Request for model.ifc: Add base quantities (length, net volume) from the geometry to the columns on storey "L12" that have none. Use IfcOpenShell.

First a look at what the model holds.

```python
import ifcopenshell
import ifcopenshell.util.element
import ifcopenshell.util.unit

model = ifcopenshell.open("model.ifc")
print(model.schema)
for unit_type in ("LENGTHUNIT", "AREAUNIT", "VOLUMEUNIT"):
    print(unit_type, ifcopenshell.util.unit.calculate_unit_scale(model, unit_type))
storey = next(s for s in model.by_type("IfcBuildingStorey") if s.Name == "L12")
columns = [e for e in ifcopenshell.util.element.get_decomposition(storey) if e.is_a("IfcColumn")]
for e in sorted(columns, key=lambda e: e.id()):
    print(e.id(), e.is_a(), e.Name, list(ifcopenshell.util.element.get_psets(e, qtos_only=True)), sep=" | ")
```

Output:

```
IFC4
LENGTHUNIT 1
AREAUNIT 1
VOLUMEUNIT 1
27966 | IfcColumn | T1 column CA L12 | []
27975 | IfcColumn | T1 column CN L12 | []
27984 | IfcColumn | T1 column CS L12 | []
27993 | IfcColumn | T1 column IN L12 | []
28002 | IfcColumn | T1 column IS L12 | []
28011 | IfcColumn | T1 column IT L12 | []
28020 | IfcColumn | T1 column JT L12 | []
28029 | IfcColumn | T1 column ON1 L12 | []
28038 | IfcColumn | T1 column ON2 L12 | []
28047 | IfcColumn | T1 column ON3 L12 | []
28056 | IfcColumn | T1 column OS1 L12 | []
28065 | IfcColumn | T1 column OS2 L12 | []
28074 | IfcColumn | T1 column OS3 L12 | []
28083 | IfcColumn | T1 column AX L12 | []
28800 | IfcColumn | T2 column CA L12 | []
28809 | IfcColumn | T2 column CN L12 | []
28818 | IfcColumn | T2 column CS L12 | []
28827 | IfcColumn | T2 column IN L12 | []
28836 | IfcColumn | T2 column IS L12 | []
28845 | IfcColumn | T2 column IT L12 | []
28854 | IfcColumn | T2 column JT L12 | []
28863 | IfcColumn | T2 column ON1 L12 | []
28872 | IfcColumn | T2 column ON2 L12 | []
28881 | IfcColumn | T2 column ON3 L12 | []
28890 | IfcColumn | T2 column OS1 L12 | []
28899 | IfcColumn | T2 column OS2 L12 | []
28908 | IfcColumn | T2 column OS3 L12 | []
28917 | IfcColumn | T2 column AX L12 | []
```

```python
import ifcopenshell
import ifcopenshell.api.pset
import ifcopenshell.geom
import ifcopenshell.util.element
import ifcopenshell.util.shape
import ifcopenshell.util.unit

model = ifcopenshell.open("model.ifc")
unit_scale = ifcopenshell.util.unit.calculate_unit_scale(model)
volume_scale = ifcopenshell.util.unit.calculate_unit_scale(model, "VOLUMEUNIT")
settings = ifcopenshell.geom.settings()

storey = next(s for s in model.by_type("IfcBuildingStorey") if s.Name == "L12")
columns = [e for e in ifcopenshell.util.element.get_decomposition(storey) if e.is_a("IfcColumn")]

for e in sorted(columns, key=lambda e: e.id()):
    if ifcopenshell.util.element.get_psets(e, qtos_only=True, should_inherit=False):
        continue
    # Geometry comes back in metres, in the element's own axes.
    shape = ifcopenshell.geom.create_shape(settings, e)
    values = {
        "Length": ifcopenshell.util.shape.get_z(shape.geometry) / unit_scale,
        "NetVolume": ifcopenshell.util.shape.get_volume(shape.geometry) / volume_scale,
    }
    qto = ifcopenshell.api.pset.add_qto(model, product=e, name="Qto_ColumnBaseQuantities")
    ifcopenshell.api.pset.edit_qto(model, qto=qto, properties=values)
    print(e.id(), {k: round(v, 3) for k, v in values.items()})

model.write("model_v2.ifc")
```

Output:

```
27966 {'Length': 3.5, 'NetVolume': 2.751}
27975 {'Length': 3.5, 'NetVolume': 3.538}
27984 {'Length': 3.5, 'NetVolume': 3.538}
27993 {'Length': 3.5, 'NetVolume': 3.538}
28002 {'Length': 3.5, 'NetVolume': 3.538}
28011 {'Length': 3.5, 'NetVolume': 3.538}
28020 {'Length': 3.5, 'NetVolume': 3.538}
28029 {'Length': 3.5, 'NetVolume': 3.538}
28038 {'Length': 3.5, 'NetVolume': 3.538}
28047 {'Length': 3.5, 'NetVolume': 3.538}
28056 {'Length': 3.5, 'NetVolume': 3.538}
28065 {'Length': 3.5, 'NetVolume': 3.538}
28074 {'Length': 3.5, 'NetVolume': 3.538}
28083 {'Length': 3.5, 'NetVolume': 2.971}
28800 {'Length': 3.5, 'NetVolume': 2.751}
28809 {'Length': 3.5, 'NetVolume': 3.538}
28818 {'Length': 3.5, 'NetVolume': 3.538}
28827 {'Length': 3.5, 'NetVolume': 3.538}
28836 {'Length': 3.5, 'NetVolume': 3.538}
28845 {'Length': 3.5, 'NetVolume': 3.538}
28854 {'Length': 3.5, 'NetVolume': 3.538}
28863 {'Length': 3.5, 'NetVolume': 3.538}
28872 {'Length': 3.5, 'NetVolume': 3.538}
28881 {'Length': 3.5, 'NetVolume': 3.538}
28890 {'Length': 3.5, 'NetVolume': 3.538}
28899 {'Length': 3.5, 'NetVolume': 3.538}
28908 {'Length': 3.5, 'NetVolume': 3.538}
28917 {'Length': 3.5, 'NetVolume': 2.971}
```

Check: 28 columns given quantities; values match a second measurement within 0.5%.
